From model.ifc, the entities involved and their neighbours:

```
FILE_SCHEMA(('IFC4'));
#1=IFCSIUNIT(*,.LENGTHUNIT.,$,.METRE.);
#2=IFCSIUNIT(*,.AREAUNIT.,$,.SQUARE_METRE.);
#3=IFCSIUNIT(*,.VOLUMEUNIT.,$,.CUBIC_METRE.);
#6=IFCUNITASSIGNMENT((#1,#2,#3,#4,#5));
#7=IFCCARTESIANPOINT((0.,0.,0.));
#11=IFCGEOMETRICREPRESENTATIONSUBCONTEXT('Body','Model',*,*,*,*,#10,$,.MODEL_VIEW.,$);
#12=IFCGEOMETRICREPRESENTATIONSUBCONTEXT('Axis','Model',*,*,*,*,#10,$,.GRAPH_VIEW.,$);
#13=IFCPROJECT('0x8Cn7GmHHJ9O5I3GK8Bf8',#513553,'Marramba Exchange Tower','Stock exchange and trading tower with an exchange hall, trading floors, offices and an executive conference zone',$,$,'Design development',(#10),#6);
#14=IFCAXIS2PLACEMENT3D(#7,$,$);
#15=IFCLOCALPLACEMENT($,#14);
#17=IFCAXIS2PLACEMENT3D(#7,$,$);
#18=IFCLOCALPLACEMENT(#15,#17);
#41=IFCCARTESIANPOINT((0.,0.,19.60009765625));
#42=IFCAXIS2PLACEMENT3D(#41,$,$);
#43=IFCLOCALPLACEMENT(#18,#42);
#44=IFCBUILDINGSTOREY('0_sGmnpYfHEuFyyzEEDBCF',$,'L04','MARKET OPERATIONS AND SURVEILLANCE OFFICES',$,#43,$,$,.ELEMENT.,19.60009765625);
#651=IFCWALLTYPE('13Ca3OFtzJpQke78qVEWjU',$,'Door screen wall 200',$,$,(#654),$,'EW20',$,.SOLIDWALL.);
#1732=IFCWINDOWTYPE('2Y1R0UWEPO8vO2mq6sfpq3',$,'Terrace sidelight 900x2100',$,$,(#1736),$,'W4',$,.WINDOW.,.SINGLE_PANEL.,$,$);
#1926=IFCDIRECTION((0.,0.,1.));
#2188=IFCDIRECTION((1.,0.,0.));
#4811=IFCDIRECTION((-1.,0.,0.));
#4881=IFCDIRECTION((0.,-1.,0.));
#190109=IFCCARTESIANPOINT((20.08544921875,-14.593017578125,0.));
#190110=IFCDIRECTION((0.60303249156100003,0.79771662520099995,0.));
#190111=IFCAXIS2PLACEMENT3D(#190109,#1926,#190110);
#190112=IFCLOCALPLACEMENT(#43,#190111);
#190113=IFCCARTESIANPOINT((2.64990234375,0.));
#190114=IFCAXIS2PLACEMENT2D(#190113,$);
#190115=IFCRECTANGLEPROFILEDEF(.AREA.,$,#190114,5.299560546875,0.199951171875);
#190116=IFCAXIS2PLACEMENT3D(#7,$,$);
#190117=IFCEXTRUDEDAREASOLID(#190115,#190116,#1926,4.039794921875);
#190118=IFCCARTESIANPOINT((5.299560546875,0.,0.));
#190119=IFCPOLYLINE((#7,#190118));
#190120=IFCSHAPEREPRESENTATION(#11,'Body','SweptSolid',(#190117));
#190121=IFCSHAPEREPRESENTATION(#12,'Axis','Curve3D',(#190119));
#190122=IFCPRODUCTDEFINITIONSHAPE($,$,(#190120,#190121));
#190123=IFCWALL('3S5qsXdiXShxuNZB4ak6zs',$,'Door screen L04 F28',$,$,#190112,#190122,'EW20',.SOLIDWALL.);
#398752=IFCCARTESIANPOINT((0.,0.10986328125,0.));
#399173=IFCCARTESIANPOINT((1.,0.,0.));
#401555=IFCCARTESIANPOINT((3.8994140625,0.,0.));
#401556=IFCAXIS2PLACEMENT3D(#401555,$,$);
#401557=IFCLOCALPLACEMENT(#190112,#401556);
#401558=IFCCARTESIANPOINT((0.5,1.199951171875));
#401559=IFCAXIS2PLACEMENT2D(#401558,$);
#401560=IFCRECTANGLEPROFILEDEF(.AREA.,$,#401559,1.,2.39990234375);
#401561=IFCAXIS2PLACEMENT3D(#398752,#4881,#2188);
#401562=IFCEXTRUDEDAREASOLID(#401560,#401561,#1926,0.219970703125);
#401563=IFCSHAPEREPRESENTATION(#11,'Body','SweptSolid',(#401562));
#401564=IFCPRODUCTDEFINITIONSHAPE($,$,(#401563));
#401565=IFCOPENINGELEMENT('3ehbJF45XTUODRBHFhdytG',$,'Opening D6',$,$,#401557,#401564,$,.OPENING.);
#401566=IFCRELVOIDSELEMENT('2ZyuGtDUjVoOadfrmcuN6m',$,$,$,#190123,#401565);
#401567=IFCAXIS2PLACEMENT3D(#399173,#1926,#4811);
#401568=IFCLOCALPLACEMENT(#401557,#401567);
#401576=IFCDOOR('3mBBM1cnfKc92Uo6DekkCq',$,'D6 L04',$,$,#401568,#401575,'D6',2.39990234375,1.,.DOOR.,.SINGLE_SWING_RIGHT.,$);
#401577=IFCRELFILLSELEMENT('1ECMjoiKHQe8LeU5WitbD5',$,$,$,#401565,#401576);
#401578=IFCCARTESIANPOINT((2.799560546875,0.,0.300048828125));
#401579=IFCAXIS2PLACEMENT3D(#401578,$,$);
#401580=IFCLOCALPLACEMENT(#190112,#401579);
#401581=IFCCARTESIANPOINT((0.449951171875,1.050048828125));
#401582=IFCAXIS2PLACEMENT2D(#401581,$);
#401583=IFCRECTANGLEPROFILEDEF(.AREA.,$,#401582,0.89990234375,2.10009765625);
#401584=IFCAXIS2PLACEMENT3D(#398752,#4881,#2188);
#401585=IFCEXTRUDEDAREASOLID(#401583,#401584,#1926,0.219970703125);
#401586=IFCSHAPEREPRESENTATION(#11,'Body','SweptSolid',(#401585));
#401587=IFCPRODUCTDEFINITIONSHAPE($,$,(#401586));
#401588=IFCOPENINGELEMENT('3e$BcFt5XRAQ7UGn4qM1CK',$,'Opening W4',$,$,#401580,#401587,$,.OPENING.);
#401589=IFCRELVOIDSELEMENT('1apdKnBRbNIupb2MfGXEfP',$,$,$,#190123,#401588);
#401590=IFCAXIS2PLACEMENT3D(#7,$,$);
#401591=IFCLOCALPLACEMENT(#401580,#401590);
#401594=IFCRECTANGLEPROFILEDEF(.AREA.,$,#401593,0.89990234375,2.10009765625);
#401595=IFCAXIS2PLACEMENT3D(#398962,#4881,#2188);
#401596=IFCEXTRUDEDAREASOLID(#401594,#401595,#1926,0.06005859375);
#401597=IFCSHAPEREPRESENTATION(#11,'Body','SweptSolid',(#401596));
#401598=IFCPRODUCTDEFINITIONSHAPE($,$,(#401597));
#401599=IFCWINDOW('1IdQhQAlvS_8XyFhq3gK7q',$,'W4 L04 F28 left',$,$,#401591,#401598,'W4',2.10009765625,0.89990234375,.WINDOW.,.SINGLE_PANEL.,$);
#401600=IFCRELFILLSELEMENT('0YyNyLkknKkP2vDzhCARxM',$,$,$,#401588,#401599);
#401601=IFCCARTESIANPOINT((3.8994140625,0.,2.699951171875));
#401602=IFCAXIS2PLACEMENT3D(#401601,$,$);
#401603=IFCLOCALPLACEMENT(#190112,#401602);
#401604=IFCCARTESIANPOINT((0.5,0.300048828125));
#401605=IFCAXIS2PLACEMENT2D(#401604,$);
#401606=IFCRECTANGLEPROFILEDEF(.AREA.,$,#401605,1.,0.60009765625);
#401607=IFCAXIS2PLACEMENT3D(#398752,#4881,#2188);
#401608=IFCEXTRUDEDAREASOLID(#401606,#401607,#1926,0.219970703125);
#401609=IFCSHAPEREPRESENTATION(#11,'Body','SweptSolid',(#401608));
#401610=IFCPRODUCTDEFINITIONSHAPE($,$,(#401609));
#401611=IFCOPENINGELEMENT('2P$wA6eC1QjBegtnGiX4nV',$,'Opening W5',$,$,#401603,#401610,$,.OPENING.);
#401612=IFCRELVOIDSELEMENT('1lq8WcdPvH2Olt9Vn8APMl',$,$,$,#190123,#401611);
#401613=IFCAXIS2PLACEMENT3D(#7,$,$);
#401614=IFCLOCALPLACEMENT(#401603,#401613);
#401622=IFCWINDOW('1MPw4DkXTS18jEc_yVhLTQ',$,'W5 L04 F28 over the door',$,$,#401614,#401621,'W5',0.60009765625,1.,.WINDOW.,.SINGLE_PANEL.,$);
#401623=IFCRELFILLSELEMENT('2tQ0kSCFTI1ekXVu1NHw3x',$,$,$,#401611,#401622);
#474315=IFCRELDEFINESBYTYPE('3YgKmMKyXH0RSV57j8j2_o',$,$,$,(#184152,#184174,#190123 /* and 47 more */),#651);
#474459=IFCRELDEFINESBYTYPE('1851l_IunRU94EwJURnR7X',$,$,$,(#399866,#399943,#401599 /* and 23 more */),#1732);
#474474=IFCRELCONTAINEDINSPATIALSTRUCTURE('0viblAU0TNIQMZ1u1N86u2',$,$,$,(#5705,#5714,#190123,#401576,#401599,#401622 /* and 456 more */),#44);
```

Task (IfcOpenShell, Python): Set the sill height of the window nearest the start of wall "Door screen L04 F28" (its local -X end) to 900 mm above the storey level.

```python
import numpy as np
import ifcopenshell
import ifcopenshell.api.geometry
import ifcopenshell.geom
import ifcopenshell.util.element
import ifcopenshell.util.placement
import ifcopenshell.util.shape
import ifcopenshell.util.unit

model = ifcopenshell.open("model.ifc")
unit_scale = ifcopenshell.util.unit.calculate_unit_scale(model)

window = model.by_guid("1IdQhQAlvS_8XyFhq3gK7q")
opening = window.FillsVoids[0].RelatingOpeningElement
storey = ifcopenshell.util.element.get_container(window, ifc_class="IfcBuildingStorey")
level = ifcopenshell.util.placement.get_local_placement(storey.ObjectPlacement)[2, 3]

# The opening's origin need not be at the sill, so measure its lowest point.
shape = ifcopenshell.geom.create_shape(ifcopenshell.geom.settings(), opening)
bottom = ifcopenshell.util.shape.get_shape_bottom_elevation(shape, shape.geometry) / unit_scale
dz = level + 0.9 / unit_scale - bottom

shift = np.array([0.0, 0.0, dz])
# The window is placed relative to its opening, so it follows when the opening moves.
matrix = ifcopenshell.util.placement.get_local_placement(opening.ObjectPlacement)
matrix[:3, 3] += shift
ifcopenshell.api.geometry.edit_object_placement(
    model, product=opening, matrix=matrix, is_si=False, should_transform_children=True
)

print(f"moved by {dz * unit_scale:+.3f} m")

model.write("model_rev.ifc")
```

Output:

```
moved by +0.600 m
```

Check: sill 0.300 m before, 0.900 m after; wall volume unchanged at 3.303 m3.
